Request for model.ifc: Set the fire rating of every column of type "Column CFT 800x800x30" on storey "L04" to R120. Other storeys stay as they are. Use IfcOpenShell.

First a look at what the model holds.

```python
import ifcopenshell
import ifcopenshell.util.element

model = ifcopenshell.open("model.ifc")
print(model.schema)
storey = next(s for s in model.by_type("IfcBuildingStorey") if s.Name == "L04")
columns = [e for e in ifcopenshell.util.element.get_decomposition(storey) if e.is_a("IfcColumn")]
seen = {}
for e in columns:
    element_type = ifcopenshell.util.element.get_type(e)
    key = (element_type.Name if element_type != e and element_type else None, ifcopenshell.util.element.get_pset(e, "Pset_ColumnCommon", "FireRating"))
    seen[key] = seen.get(key, 0) + 1
for (name, value), count in sorted(seen.items(), key=str):
    print(count, "x", name, "|", value)
```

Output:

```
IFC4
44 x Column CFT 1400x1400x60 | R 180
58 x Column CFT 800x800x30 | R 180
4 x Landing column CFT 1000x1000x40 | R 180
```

```python
import ifcopenshell
import ifcopenshell.api.pset
import ifcopenshell.util.element

model = ifcopenshell.open("model.ifc")

storey = next(s for s in model.by_type("IfcBuildingStorey") if s.Name == "L04")
columns = [e for e in ifcopenshell.util.element.get_decomposition(storey) if e.is_a("IfcColumn")]

count = 0
for e in columns:
    element_type = ifcopenshell.util.element.get_type(e)
    if element_type in (None, e) or element_type.Name != "Column CFT 800x800x30":
        continue
    found = ifcopenshell.util.element.get_pset(e, "Pset_ColumnCommon", should_inherit=False)
    if found:
        pset = model.by_id(found["id"])
        if len(ifcopenshell.util.element.get_elements_by_pset(pset)) > 1:
            pset = ifcopenshell.api.pset.unshare_pset(model, products=[e], pset=pset)[0]
    else:
        pset = ifcopenshell.api.pset.add_pset(model, product=e, name="Pset_ColumnCommon")
    ifcopenshell.api.pset.edit_pset(model, pset=pset, properties={"FireRating": "R120"})
    count += 1

print(count, "columns updated")

model.write("model_updated.ifc")
```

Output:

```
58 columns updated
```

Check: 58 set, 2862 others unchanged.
